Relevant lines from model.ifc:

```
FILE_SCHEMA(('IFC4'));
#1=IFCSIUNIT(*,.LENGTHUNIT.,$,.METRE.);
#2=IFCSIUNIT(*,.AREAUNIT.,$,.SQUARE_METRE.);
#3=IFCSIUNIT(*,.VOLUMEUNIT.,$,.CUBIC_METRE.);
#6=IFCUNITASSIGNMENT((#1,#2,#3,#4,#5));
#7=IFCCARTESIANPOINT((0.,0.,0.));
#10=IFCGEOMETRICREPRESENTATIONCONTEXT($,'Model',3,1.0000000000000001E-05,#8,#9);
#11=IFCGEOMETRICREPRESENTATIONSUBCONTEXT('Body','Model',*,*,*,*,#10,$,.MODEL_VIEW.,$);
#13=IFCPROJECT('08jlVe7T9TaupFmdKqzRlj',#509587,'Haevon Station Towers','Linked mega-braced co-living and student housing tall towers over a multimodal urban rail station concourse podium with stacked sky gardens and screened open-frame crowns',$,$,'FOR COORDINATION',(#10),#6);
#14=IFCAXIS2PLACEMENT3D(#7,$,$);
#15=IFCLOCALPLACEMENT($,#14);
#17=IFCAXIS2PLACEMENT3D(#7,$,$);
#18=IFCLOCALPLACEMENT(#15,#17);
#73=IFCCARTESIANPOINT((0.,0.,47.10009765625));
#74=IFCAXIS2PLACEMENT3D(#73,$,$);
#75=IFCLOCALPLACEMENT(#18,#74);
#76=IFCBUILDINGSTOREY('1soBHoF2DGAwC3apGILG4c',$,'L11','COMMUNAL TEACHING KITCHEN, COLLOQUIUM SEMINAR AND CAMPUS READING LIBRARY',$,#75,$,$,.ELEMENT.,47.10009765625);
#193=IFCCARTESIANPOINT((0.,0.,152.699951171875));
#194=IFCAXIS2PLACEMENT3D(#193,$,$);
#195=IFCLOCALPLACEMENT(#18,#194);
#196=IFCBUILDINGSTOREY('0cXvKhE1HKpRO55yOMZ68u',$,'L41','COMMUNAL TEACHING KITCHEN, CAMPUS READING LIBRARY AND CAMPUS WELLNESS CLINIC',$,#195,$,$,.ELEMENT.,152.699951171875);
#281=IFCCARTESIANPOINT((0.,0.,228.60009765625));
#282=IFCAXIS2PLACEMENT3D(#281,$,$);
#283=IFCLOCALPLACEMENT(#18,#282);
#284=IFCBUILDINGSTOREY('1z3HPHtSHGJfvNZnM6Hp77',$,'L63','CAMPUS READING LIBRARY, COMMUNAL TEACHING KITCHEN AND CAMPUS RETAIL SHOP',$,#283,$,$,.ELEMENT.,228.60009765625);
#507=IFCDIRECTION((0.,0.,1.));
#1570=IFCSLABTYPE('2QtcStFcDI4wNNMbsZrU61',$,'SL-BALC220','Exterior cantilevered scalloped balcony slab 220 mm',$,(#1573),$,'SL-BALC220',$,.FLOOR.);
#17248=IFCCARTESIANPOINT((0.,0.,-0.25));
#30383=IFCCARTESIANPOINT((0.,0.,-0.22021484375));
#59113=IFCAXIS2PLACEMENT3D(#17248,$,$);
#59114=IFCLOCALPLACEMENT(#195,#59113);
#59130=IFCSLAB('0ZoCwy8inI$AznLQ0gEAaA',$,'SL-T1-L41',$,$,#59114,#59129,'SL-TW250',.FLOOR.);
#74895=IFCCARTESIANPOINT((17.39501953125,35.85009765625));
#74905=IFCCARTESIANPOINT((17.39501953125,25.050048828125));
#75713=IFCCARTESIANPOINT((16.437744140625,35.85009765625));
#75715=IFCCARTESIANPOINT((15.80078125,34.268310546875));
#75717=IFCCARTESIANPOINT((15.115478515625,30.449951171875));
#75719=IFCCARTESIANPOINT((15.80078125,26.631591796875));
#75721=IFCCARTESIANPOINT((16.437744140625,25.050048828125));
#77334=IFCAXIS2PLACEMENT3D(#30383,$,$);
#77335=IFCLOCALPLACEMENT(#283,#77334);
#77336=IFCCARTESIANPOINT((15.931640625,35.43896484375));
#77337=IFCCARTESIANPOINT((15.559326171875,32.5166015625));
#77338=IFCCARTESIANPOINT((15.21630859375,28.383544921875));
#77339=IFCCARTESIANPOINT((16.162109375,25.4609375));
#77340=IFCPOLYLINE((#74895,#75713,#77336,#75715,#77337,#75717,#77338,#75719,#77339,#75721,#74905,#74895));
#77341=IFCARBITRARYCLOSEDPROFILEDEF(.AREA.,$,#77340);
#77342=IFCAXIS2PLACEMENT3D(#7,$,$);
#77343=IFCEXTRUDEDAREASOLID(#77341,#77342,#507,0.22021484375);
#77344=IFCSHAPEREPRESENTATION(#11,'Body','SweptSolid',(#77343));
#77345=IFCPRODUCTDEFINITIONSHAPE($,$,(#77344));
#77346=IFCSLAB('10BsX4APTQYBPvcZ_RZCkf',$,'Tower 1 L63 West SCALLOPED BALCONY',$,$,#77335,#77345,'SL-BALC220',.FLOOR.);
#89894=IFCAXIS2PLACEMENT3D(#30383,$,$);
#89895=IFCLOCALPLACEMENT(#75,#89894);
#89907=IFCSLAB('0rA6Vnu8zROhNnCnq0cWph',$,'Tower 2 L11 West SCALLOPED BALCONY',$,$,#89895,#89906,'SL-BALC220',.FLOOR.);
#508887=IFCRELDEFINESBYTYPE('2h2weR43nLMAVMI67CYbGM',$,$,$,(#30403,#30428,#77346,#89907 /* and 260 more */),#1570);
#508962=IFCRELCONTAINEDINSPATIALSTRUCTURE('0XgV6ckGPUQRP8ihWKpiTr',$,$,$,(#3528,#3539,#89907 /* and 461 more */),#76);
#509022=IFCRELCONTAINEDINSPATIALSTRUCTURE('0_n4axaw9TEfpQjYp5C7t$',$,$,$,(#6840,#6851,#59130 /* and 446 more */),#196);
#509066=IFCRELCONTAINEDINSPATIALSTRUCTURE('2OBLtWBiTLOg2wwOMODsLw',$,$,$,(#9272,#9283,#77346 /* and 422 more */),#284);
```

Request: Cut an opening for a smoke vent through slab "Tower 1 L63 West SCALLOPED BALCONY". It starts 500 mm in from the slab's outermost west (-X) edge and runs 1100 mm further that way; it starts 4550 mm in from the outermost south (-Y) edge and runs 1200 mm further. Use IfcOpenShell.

```python
import numpy as np
import ifcopenshell
import ifcopenshell.api.feature
import ifcopenshell.api.geometry
import ifcopenshell.api.root
import ifcopenshell.geom
import ifcopenshell.util.placement
import ifcopenshell.util.representation
import ifcopenshell.util.shape
import ifcopenshell.util.unit

model = ifcopenshell.open("model.ifc")
unit_scale = ifcopenshell.util.unit.calculate_unit_scale(model)
settings = ifcopenshell.geom.settings()


def volume(element):
    """Net volume in cubic metres, openings subtracted."""
    shape = ifcopenshell.geom.create_shape(settings, element)
    return ifcopenshell.util.shape.get_volume(shape.geometry)


slab = model.by_id(77346)
before = volume(slab)

# Extent in the slab's own axes, in metres. The edges named are its -X and -Y sides.
slab_shape = ifcopenshell.geom.create_shape(settings, slab)
vertices = ifcopenshell.util.shape.get_vertices(slab_shape.geometry)
x_min, y_min, bottom = vertices.min(axis=0)
top = vertices[:, 2].max()

opening = ifcopenshell.api.root.create_entity(model, ifc_class="IfcOpeningElement", name="Smoke vent opening", predefined_type="OPENING")
context = ifcopenshell.util.representation.get_context(model, "Model", "Body", "MODEL_VIEW")
width, depth = 1.1, 1.2
outline = [(0.0, 0.0), (width, 0.0), (width, depth), (0.0, depth), (0.0, 0.0)]
# Overshoot both faces by 50 mm so the cut is clean.
shape = ifcopenshell.api.geometry.add_slab_representation(
    model, context=context, depth=top - bottom + 0.1, polyline=outline
)
ifcopenshell.api.geometry.assign_representation(model, product=opening, representation=shape)

matrix = ifcopenshell.util.placement.get_local_placement(slab.ObjectPlacement)
matrix[:, 3] = matrix @ np.append(np.array([x_min + 0.5, y_min + 4.55, bottom - 0.05]) / unit_scale, 1.0)
ifcopenshell.api.geometry.edit_object_placement(model, product=opening, matrix=matrix, is_si=False)
ifcopenshell.api.feature.add_feature(model, feature=opening, element=slab)

after = volume(slab)

print(f"slab volume {before:.3f} -> {after:.3f} m3")

model.write("model_edited.ifc")
```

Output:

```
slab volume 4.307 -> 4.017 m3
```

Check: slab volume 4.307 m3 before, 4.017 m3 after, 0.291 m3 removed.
